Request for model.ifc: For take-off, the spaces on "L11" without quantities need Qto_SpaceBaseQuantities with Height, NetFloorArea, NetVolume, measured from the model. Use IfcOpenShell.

First a look at what the model holds.

```python
import ifcopenshell
import ifcopenshell.util.element
import ifcopenshell.util.unit

model = ifcopenshell.open("model.ifc")
print(model.schema)
for unit_type in ("LENGTHUNIT", "AREAUNIT", "VOLUMEUNIT"):
    print(unit_type, ifcopenshell.util.unit.calculate_unit_scale(model, unit_type))
storey = next(s for s in model.by_type("IfcBuildingStorey") if s.Name == "L11")
spaces = [e for e in ifcopenshell.util.element.get_decomposition(storey) if e.is_a("IfcSpace")]
for e in sorted(spaces, key=lambda e: e.id()):
    print(e.id(), e.is_a(), e.Name, list(ifcopenshell.util.element.get_psets(e, qtos_only=True)), sep=" | ")
```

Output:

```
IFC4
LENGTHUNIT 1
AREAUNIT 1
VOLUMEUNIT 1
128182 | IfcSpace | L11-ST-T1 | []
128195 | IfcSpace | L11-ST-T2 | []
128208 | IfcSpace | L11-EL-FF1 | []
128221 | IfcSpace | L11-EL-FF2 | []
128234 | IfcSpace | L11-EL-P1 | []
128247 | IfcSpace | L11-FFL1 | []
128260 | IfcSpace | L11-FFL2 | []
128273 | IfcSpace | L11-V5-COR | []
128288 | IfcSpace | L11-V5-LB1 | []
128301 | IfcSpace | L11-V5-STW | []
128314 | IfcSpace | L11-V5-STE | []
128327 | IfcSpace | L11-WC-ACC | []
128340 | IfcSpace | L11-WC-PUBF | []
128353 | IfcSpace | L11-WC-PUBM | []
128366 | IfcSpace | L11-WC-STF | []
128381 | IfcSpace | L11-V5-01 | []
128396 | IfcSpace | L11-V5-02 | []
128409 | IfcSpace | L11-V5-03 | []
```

```python
import ifcopenshell
import ifcopenshell.api.pset
import ifcopenshell.geom
import ifcopenshell.util.element
import ifcopenshell.util.shape
import ifcopenshell.util.unit

model = ifcopenshell.open("model.ifc")
unit_scale = ifcopenshell.util.unit.calculate_unit_scale(model)
area_scale = ifcopenshell.util.unit.calculate_unit_scale(model, "AREAUNIT")
volume_scale = ifcopenshell.util.unit.calculate_unit_scale(model, "VOLUMEUNIT")
settings = ifcopenshell.geom.settings()

storey = next(s for s in model.by_type("IfcBuildingStorey") if s.Name == "L11")
spaces = [e for e in ifcopenshell.util.element.get_decomposition(storey) if e.is_a("IfcSpace")]

for e in sorted(spaces, key=lambda e: e.id()):
    if ifcopenshell.util.element.get_psets(e, qtos_only=True, should_inherit=False):
        continue
    # Geometry comes back in metres, in the element's own axes.
    shape = ifcopenshell.geom.create_shape(settings, e)
    values = {
        "Height": ifcopenshell.util.shape.get_z(shape.geometry) / unit_scale,
        "NetFloorArea": ifcopenshell.util.shape.get_footprint_area(shape.geometry) / area_scale,
        "NetVolume": ifcopenshell.util.shape.get_volume(shape.geometry) / volume_scale,
    }
    qto = ifcopenshell.api.pset.add_qto(model, product=e, name="Qto_SpaceBaseQuantities")
    ifcopenshell.api.pset.edit_qto(model, qto=qto, properties=values)
    print(e.id(), {k: round(v, 3) for k, v in values.items()})

model.write("model-out.ifc")
```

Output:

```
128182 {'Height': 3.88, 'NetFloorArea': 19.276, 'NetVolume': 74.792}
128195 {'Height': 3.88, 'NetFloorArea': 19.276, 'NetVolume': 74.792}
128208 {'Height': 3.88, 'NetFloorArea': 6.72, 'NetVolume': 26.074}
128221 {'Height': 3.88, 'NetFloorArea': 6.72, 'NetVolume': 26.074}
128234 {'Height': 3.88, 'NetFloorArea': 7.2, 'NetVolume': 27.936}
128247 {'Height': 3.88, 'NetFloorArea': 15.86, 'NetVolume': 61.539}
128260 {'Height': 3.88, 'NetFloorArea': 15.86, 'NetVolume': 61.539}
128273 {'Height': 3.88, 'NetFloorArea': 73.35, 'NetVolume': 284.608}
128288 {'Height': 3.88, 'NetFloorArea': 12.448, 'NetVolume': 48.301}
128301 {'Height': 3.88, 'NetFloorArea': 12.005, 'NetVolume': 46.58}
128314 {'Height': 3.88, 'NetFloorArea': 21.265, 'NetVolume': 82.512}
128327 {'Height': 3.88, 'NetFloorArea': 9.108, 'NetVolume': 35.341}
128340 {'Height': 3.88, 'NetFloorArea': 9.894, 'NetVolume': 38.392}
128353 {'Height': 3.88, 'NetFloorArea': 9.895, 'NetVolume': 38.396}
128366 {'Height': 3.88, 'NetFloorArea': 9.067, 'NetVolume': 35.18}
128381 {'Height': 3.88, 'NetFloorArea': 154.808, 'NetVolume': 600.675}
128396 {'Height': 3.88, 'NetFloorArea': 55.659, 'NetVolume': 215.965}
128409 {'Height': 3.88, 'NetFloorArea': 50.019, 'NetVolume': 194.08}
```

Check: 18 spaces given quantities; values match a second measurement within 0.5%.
